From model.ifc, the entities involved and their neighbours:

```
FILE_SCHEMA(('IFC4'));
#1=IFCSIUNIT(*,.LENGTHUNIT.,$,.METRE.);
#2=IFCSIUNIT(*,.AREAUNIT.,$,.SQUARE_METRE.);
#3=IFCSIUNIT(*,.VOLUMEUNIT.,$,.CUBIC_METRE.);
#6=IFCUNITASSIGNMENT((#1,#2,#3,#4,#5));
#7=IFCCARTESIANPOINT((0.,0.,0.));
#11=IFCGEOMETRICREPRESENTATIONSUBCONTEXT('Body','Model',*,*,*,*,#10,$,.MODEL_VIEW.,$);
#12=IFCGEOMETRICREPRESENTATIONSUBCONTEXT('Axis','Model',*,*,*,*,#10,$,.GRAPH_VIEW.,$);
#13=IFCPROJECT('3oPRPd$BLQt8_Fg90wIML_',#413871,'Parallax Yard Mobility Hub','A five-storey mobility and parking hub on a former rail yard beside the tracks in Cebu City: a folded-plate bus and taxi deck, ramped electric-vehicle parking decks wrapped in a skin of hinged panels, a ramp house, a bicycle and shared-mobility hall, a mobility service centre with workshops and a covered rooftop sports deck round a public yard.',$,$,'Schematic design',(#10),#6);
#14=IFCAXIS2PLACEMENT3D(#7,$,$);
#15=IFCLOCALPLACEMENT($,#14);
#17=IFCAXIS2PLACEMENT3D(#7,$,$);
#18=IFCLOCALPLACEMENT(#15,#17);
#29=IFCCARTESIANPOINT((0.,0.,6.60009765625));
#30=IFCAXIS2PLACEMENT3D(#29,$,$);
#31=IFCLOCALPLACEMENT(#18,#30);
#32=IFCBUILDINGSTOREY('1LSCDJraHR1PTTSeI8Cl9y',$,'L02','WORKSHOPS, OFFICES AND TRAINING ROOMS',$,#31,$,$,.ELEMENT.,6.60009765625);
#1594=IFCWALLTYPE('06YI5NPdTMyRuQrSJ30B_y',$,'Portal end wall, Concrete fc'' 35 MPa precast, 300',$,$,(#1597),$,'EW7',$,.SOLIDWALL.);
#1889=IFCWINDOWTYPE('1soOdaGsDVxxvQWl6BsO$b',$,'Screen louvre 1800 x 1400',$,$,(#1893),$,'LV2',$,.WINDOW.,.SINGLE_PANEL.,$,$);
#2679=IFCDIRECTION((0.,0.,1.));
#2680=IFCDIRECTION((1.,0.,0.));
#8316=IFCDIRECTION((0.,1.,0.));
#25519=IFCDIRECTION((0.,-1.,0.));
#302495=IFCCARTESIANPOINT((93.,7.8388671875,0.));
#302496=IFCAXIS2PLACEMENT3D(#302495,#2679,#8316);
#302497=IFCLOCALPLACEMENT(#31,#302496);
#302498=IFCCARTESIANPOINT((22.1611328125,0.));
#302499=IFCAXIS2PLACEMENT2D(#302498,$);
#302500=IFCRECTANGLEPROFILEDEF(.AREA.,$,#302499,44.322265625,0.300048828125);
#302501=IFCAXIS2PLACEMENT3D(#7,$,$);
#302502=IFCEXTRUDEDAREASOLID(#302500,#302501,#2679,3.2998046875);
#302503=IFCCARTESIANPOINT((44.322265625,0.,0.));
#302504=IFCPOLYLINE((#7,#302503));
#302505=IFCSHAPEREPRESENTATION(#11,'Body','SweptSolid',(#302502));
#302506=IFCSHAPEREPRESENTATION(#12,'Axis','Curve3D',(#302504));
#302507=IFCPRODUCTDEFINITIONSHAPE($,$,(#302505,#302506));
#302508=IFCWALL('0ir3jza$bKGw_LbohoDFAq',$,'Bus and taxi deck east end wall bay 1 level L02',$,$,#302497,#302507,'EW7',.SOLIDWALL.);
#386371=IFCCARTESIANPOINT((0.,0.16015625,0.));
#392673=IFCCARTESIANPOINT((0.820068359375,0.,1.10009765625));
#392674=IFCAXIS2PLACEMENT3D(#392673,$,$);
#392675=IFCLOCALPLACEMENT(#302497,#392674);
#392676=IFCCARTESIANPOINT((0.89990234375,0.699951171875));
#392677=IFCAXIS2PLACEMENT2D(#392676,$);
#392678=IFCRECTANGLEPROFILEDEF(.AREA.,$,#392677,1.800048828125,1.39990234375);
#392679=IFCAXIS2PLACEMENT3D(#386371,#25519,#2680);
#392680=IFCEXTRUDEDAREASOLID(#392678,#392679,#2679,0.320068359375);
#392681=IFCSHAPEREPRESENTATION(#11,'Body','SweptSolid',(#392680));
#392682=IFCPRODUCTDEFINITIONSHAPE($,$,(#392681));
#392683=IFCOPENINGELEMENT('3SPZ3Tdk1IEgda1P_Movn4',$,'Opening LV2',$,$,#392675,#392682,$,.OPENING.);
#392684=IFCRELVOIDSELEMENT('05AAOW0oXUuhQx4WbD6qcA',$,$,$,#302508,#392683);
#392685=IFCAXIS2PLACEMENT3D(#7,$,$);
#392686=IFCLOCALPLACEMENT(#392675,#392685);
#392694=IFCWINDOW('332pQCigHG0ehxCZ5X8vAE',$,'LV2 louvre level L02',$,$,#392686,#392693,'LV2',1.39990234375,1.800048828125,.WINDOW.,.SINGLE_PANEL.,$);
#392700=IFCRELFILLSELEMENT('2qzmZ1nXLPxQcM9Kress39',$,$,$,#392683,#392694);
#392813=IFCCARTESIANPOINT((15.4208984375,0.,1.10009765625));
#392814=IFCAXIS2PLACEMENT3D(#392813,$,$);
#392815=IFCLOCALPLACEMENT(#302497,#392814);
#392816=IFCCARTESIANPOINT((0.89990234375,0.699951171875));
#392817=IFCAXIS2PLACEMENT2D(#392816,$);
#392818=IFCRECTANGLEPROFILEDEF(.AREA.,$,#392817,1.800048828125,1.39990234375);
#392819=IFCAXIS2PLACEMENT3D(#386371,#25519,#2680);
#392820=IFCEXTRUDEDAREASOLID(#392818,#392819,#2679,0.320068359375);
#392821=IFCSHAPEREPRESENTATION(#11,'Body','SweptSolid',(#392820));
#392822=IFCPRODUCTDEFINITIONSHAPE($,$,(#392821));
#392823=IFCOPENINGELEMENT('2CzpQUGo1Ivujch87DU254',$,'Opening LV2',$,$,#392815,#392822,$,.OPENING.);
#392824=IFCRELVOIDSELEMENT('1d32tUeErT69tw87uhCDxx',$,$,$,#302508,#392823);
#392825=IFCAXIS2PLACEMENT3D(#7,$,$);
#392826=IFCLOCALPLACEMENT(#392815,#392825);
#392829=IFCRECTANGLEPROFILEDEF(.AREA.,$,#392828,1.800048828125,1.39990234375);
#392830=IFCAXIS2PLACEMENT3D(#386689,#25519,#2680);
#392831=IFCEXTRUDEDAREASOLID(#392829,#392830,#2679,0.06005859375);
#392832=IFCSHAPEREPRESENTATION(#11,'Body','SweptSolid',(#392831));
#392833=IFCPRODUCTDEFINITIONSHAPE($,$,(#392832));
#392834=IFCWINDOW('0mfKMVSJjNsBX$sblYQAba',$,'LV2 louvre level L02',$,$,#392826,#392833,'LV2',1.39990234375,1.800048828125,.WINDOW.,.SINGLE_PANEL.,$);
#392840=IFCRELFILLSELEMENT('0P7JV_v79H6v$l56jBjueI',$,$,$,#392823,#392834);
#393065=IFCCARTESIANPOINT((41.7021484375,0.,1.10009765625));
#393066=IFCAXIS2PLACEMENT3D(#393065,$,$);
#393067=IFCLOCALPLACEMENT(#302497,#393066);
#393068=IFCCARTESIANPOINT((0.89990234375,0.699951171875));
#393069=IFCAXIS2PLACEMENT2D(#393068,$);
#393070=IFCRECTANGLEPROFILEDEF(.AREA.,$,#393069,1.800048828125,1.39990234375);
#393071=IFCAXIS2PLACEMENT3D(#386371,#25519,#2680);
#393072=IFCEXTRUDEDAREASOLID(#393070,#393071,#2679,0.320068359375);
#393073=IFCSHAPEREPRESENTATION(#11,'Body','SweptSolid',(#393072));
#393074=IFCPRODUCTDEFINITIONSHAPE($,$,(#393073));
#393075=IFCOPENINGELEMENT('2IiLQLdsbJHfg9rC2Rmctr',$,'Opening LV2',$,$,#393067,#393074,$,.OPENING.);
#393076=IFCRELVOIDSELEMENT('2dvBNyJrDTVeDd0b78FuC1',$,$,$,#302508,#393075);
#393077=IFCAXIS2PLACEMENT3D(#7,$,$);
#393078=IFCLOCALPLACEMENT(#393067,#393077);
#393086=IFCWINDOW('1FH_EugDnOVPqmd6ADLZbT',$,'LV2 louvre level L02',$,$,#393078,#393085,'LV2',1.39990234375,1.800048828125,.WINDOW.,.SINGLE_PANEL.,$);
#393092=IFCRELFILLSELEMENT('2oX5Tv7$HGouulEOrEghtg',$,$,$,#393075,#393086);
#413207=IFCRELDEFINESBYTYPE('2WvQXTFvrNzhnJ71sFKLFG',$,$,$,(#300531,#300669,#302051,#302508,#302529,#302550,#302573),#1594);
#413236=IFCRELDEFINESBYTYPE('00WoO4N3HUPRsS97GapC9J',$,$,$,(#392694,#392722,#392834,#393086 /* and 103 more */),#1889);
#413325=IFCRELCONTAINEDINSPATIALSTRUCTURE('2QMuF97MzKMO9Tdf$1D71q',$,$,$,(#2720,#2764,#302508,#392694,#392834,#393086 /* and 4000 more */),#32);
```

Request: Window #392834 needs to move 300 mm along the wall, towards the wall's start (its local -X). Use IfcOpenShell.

```python
import ifcopenshell
import ifcopenshell.api.geometry
import ifcopenshell.util.placement
import ifcopenshell.util.unit

model = ifcopenshell.open("model.ifc")
unit_scale = ifcopenshell.util.unit.calculate_unit_scale(model)

window = model.by_id(392834)
opening = window.FillsVoids[0].RelatingOpeningElement
wall = opening.VoidsElements[0].RelatingBuildingElement

wall_matrix = ifcopenshell.util.placement.get_local_placement(wall.ObjectPlacement)
shift = wall_matrix[:3, 0] * -0.3 / unit_scale
before = ifcopenshell.util.placement.get_local_placement(window.ObjectPlacement)[:3, 3].copy()

# The window is placed relative to its opening, so it follows when the opening moves.
matrix = ifcopenshell.util.placement.get_local_placement(opening.ObjectPlacement)
matrix[:3, 3] += shift
ifcopenshell.api.geometry.edit_object_placement(
    model, product=opening, matrix=matrix, is_si=False, should_transform_children=True
)

after = ifcopenshell.util.placement.get_local_placement(window.ObjectPlacement)[:3, 3]
print("window moved by", (after - before).round(3) + 0.0)

model.write("model_updated.ifc")
```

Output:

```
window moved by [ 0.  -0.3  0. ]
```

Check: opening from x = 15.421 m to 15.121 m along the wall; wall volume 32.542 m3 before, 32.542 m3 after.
